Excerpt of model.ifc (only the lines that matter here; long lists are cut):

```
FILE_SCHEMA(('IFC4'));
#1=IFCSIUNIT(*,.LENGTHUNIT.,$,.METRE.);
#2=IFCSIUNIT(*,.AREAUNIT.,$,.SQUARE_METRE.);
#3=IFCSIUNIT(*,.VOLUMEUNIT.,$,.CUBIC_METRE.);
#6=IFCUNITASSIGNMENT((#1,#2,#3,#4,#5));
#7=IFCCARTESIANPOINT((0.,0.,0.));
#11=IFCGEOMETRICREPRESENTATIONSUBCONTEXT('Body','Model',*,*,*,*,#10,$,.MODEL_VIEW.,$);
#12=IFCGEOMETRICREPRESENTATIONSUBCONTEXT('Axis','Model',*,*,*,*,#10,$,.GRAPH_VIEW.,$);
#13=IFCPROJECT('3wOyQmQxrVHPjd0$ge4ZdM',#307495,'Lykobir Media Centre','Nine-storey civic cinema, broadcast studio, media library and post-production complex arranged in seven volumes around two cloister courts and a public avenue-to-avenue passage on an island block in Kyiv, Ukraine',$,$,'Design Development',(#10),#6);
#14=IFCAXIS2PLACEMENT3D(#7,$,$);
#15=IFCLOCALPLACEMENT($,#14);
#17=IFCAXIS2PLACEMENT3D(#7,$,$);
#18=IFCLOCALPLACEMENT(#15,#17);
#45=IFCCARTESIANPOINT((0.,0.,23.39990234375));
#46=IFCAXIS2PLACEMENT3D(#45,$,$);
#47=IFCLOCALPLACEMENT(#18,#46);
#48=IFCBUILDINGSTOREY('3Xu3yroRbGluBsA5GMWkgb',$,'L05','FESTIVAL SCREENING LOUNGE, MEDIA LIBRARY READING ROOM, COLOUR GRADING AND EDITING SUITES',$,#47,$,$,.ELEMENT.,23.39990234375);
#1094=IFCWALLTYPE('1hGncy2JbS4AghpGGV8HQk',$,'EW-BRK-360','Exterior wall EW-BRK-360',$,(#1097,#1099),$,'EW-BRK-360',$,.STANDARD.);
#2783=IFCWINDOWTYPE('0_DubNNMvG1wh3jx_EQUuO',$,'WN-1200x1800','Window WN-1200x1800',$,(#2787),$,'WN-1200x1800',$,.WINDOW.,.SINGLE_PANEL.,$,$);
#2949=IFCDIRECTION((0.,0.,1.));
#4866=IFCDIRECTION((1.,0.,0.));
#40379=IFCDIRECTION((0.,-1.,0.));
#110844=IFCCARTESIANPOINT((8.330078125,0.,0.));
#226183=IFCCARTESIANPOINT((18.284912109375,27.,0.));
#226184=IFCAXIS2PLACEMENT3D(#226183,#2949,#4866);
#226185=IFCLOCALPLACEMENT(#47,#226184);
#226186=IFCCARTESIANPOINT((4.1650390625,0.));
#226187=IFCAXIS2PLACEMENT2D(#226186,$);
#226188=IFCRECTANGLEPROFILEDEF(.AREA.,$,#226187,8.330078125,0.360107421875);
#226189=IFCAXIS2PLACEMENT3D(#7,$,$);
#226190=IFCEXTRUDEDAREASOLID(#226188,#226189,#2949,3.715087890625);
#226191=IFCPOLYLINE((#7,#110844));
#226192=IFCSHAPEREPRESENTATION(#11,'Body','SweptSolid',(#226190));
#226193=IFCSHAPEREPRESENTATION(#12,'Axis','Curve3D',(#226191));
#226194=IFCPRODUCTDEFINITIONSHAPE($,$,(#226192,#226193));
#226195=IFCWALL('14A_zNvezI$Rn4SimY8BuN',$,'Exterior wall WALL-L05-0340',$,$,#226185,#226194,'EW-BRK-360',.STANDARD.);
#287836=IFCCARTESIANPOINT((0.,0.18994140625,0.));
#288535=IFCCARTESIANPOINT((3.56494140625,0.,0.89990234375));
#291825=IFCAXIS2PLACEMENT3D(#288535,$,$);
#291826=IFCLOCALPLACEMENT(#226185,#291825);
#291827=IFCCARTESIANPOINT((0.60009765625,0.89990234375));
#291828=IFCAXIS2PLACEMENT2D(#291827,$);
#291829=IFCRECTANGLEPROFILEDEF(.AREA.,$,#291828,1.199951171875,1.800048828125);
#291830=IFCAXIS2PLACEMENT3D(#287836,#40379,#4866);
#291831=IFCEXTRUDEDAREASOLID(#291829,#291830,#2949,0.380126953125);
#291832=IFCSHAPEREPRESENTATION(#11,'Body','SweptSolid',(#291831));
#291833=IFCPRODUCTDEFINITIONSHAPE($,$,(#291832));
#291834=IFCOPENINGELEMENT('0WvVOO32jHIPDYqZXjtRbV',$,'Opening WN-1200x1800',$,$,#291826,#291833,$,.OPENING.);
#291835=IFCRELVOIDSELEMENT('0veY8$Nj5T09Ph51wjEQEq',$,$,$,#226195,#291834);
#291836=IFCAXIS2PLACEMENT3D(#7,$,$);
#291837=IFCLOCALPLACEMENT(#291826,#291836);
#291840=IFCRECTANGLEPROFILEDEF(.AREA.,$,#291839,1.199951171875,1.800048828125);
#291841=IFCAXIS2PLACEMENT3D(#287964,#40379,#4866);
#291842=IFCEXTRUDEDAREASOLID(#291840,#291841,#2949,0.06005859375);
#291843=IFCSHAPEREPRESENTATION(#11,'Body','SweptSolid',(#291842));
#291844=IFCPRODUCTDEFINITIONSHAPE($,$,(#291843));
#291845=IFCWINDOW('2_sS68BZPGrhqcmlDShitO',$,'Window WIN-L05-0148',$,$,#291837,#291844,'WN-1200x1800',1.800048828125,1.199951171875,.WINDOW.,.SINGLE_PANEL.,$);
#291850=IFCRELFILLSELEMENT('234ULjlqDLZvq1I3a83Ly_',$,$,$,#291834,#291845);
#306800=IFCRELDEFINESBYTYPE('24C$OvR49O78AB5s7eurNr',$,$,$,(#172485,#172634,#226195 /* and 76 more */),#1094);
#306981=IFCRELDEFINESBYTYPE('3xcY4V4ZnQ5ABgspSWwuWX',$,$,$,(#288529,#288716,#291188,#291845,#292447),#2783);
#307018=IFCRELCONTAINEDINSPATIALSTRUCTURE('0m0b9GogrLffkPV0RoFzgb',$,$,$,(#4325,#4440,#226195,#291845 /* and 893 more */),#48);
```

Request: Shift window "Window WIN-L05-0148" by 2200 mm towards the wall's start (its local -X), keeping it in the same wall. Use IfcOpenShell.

```python
import ifcopenshell
import ifcopenshell.api.geometry
import ifcopenshell.util.placement
import ifcopenshell.util.unit

model = ifcopenshell.open("model.ifc")
unit_scale = ifcopenshell.util.unit.calculate_unit_scale(model)

window = model.by_guid("2_sS68BZPGrhqcmlDShitO")
opening = window.FillsVoids[0].RelatingOpeningElement
wall = opening.VoidsElements[0].RelatingBuildingElement

wall_matrix = ifcopenshell.util.placement.get_local_placement(wall.ObjectPlacement)
shift = wall_matrix[:3, 0] * -2.2 / unit_scale
before = ifcopenshell.util.placement.get_local_placement(window.ObjectPlacement)[:3, 3].copy()

# The window is placed relative to its opening, so it follows when the opening moves.
matrix = ifcopenshell.util.placement.get_local_placement(opening.ObjectPlacement)
matrix[:3, 3] += shift
ifcopenshell.api.geometry.edit_object_placement(
    model, product=opening, matrix=matrix, is_si=False, should_transform_children=True
)

after = ifcopenshell.util.placement.get_local_placement(window.ObjectPlacement)[:3, 3]
print("window moved by", (after - before).round(3) + 0.0)

model.write("model_rev.ifc")
```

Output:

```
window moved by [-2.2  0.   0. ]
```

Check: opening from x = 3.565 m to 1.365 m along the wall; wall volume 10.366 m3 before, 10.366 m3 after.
